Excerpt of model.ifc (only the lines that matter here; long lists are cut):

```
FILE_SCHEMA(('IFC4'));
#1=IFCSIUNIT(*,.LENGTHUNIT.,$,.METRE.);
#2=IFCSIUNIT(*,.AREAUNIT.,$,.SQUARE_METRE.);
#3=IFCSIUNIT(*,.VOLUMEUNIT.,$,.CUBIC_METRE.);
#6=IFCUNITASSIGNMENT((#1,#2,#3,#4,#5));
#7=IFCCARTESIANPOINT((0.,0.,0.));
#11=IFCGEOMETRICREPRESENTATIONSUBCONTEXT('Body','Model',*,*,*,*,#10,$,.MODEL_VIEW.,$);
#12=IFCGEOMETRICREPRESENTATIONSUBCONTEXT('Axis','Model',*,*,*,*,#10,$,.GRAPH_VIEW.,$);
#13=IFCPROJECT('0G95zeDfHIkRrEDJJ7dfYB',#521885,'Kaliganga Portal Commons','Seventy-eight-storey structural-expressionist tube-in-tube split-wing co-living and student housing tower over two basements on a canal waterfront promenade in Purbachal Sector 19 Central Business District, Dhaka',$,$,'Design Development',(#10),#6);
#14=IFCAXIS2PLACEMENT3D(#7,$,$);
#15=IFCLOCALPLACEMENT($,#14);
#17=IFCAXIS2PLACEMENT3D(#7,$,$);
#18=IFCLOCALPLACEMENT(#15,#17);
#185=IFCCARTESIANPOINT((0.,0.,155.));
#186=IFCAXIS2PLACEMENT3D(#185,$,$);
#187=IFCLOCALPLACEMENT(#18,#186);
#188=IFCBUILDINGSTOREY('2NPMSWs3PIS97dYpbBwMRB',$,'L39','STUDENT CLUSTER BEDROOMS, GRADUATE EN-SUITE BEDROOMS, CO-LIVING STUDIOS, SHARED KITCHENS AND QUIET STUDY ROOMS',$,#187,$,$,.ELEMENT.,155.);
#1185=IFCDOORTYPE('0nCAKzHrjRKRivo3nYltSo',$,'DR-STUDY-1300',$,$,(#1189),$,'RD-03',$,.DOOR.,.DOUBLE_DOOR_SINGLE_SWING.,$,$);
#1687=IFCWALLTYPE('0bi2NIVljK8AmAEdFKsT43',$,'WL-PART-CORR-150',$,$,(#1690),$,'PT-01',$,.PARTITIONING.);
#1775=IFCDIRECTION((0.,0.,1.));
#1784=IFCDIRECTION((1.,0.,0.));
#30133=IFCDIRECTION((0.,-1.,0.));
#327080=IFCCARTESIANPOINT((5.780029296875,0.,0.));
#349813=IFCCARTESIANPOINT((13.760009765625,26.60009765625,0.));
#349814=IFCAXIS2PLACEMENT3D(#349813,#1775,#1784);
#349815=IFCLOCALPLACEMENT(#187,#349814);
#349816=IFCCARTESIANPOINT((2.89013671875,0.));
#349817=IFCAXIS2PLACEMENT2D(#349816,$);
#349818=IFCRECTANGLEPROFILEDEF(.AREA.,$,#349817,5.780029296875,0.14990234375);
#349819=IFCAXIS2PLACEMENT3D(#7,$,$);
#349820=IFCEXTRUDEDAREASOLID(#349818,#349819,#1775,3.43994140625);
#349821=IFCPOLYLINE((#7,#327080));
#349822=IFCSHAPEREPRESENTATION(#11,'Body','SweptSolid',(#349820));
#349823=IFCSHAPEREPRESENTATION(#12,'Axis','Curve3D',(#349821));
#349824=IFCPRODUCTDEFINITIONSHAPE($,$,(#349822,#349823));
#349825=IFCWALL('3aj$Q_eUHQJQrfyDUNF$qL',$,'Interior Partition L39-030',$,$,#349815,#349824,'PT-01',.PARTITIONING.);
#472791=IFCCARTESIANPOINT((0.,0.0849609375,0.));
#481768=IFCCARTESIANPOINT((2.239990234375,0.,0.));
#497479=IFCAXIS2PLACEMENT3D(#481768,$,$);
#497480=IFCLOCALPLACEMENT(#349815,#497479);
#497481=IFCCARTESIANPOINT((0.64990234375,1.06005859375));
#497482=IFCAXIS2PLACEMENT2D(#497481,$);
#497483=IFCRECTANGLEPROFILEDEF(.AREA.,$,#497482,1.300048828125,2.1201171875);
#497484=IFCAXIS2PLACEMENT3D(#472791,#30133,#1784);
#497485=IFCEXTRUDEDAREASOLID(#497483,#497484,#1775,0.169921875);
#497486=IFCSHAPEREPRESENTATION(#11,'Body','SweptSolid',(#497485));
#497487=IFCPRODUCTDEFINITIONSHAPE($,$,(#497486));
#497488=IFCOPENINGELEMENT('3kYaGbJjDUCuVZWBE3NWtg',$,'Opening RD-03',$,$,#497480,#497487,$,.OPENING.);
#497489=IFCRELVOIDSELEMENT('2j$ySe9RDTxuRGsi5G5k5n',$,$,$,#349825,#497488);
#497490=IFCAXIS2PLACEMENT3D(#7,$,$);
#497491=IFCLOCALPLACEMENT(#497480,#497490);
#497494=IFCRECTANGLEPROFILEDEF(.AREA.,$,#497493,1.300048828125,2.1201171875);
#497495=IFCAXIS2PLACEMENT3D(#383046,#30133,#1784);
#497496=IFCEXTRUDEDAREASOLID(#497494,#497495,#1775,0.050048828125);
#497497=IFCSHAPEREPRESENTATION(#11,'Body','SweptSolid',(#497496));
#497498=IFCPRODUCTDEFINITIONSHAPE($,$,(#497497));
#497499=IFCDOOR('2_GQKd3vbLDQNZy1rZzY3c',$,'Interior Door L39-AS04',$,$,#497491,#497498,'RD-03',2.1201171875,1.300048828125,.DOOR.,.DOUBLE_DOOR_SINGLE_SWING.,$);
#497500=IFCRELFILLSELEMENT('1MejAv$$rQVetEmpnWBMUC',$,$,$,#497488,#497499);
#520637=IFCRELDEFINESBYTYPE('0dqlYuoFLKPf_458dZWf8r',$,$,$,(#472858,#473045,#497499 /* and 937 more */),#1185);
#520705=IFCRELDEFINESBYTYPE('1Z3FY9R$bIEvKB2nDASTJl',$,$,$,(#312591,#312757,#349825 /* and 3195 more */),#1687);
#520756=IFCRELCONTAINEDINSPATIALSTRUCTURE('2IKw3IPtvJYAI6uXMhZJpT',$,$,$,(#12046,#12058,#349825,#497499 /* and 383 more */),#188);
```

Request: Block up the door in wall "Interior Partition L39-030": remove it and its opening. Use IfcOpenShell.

```python
import ifcopenshell
import ifcopenshell.api.feature
import ifcopenshell.api.root
import ifcopenshell.geom
import ifcopenshell.util.shape

model = ifcopenshell.open("model.ifc")
settings = ifcopenshell.geom.settings()


def volume(element):
    """Net volume in cubic metres, openings subtracted."""
    shape = ifcopenshell.geom.create_shape(settings, element)
    return ifcopenshell.util.shape.get_volume(shape.geometry)


door = model.by_id(497499)
opening = door.FillsVoids[0].RelatingOpeningElement
wall = opening.VoidsElements[0].RelatingBuildingElement
before = volume(wall)

ifcopenshell.api.root.remove_product(model, product=door)
ifcopenshell.api.feature.remove_feature(model, feature=opening)

after = volume(wall)

print(f"wall volume {before:.3f} -> {after:.3f} m3")

model.write("model_v2.ifc")
```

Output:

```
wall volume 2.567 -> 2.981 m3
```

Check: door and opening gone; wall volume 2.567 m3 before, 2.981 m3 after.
